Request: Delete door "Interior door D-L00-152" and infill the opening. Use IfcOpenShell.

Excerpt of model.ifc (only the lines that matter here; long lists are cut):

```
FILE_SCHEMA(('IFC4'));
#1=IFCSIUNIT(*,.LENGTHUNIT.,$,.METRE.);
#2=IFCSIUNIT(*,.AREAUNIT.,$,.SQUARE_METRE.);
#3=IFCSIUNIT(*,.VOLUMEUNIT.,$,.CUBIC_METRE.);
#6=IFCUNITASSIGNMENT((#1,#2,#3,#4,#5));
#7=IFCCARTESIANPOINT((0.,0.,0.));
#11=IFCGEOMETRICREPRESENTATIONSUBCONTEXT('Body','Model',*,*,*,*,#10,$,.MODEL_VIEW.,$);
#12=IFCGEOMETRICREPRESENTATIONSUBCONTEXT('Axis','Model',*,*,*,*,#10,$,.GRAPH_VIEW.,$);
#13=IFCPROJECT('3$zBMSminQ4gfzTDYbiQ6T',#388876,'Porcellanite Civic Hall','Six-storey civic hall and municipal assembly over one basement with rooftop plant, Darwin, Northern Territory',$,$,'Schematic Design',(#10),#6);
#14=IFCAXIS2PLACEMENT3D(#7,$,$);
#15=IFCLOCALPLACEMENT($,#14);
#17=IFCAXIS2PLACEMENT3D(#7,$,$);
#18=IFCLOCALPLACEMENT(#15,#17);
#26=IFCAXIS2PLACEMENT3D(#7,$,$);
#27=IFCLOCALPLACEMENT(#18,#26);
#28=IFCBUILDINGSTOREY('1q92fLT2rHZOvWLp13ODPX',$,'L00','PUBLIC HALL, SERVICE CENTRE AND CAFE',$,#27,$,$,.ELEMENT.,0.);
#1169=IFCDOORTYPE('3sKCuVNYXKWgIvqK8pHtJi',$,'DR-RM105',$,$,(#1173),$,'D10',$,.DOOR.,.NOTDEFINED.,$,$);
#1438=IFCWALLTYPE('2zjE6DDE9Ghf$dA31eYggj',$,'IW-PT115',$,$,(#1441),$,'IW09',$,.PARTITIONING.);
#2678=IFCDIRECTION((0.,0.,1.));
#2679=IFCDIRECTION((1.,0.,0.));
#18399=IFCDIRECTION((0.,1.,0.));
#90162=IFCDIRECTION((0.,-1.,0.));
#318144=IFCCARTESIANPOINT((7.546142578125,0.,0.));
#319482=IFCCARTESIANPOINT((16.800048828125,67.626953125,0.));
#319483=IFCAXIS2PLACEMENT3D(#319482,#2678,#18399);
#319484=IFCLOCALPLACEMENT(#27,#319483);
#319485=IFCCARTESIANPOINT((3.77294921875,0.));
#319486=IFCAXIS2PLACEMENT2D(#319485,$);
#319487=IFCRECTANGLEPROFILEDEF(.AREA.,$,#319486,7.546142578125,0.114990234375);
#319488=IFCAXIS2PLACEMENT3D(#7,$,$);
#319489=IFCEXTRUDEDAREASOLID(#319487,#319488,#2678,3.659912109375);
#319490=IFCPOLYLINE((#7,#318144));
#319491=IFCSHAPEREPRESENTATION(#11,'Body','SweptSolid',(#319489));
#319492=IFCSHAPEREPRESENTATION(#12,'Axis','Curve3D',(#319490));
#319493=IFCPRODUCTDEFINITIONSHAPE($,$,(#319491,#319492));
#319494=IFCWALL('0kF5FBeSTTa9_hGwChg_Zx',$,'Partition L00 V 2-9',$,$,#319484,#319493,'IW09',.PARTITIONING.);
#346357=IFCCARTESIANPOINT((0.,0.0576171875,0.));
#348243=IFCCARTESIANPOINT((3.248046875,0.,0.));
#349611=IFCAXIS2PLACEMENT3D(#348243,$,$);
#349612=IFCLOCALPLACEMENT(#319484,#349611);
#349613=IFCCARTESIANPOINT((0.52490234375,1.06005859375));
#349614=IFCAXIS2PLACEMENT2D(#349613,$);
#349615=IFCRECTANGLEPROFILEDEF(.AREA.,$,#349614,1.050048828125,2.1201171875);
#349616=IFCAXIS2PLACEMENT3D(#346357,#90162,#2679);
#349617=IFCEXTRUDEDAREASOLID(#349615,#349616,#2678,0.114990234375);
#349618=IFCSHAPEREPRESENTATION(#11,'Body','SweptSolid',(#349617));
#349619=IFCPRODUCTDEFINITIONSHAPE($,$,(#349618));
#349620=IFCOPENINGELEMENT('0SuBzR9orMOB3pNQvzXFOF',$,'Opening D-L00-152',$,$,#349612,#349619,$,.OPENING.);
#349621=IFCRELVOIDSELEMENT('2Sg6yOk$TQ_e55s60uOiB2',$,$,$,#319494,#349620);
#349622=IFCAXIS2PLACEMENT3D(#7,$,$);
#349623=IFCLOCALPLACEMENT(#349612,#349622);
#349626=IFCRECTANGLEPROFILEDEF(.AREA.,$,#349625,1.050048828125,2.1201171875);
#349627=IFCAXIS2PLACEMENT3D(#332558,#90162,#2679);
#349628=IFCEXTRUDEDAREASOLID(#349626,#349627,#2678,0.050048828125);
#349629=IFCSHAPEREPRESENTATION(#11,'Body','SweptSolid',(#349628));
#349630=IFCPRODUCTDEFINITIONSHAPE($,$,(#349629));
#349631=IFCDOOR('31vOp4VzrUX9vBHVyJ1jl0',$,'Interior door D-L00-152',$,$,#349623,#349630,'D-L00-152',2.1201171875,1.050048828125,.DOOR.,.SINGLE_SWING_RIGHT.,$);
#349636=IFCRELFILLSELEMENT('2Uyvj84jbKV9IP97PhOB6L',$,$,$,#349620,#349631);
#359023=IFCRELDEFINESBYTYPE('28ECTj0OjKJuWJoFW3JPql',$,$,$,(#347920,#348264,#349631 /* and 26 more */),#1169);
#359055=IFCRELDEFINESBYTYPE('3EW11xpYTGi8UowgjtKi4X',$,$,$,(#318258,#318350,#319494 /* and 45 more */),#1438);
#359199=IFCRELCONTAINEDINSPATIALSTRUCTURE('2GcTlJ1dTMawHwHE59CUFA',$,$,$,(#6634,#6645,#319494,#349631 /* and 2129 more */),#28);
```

```python
import ifcopenshell
import ifcopenshell.api.feature
import ifcopenshell.api.root
import ifcopenshell.geom
import ifcopenshell.util.shape

model = ifcopenshell.open("model.ifc")
settings = ifcopenshell.geom.settings()


def volume(element):
    """Net volume in cubic metres, openings subtracted."""
    shape = ifcopenshell.geom.create_shape(settings, element)
    return ifcopenshell.util.shape.get_volume(shape.geometry)


door = model.by_guid("31vOp4VzrUX9vBHVyJ1jl0")
opening = door.FillsVoids[0].RelatingOpeningElement
wall = opening.VoidsElements[0].RelatingBuildingElement
before = volume(wall)

ifcopenshell.api.root.remove_product(model, product=door)
ifcopenshell.api.feature.remove_feature(model, feature=opening)

after = volume(wall)

print(f"wall volume {before:.3f} -> {after:.3f} m3")

model.write("model_edited.ifc")
```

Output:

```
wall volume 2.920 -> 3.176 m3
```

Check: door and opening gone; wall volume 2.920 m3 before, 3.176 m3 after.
